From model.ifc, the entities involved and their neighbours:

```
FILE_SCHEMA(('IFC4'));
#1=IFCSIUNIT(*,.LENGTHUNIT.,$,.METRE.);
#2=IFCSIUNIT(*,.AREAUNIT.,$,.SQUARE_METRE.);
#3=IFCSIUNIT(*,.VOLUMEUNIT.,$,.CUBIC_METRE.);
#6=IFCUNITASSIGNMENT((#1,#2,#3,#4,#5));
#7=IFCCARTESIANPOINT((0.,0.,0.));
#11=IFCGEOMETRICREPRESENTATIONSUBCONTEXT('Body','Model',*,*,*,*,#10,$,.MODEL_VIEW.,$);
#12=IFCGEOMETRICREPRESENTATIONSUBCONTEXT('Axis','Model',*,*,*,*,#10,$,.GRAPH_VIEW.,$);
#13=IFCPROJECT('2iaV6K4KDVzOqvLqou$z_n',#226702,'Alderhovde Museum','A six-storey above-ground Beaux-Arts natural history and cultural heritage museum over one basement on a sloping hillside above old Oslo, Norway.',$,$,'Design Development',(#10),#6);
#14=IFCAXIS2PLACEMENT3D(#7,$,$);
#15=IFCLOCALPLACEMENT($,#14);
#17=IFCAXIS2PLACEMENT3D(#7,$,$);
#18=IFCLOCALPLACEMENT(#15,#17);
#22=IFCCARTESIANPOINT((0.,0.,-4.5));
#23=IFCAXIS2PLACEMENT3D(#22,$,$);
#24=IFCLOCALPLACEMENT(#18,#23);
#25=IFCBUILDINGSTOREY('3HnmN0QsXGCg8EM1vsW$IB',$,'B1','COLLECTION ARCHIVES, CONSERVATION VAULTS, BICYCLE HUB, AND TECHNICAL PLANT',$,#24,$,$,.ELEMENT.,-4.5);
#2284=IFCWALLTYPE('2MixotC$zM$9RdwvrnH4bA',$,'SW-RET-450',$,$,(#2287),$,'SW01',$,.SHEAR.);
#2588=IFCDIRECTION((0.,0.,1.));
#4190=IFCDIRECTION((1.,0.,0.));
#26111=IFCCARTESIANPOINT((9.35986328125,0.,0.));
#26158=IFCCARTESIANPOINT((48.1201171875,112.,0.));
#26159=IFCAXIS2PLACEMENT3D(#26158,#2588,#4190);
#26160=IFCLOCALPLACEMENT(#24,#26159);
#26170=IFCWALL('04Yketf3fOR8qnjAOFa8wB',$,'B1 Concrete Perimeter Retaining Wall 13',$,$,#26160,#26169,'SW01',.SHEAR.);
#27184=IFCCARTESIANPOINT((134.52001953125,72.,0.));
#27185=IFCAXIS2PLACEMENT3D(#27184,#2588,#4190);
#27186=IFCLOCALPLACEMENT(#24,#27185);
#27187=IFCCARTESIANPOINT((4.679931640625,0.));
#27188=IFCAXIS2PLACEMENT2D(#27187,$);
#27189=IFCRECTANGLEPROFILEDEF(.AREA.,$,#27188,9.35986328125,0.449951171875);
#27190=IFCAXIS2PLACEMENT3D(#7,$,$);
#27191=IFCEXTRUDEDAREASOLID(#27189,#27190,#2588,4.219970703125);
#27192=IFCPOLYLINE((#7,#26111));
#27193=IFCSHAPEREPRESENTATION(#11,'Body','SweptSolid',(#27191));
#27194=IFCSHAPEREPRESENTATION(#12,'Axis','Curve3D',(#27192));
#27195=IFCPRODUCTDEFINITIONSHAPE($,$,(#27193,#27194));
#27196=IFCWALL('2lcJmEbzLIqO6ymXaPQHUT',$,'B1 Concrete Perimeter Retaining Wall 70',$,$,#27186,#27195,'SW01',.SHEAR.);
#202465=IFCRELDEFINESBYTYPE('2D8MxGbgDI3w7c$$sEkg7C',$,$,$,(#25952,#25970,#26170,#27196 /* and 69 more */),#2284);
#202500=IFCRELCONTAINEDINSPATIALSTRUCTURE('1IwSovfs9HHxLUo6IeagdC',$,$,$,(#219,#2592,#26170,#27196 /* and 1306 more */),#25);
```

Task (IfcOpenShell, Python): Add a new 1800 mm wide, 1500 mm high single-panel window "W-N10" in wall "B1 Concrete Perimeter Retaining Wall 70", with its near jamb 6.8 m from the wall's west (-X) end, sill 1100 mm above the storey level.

```python
import numpy as np
import ifcopenshell
import ifcopenshell.api.feature
import ifcopenshell.api.geometry
import ifcopenshell.api.root
import ifcopenshell.api.spatial
import ifcopenshell.geom
import ifcopenshell.util.element
import ifcopenshell.util.placement
import ifcopenshell.util.representation
import ifcopenshell.util.shape
import ifcopenshell.util.unit

model = ifcopenshell.open("model.ifc")
unit_scale = ifcopenshell.util.unit.calculate_unit_scale(model)
settings = ifcopenshell.geom.settings()


def volume(element):
    """Net volume in cubic metres, openings subtracted."""
    shape = ifcopenshell.geom.create_shape(settings, element)
    return ifcopenshell.util.shape.get_volume(shape.geometry)


wall = model.by_guid("2lcJmEbzLIqO6ymXaPQHUT")
storey = ifcopenshell.util.element.get_container(wall, ifc_class="IfcBuildingStorey")
context = ifcopenshell.util.representation.get_context(model, "Model", "Body", "MODEL_VIEW")
before = volume(wall)

width, height, from_end, sill = 1.8, 1.5, 6.8, 1.1  # metres

# The wall runs along its own X axis, and the end named is its -X end.
wall_shape = ifcopenshell.geom.create_shape(settings, wall)
x, y, z = ifcopenshell.util.shape.get_vertices(wall_shape.geometry).T
start = x.min() + from_end
face, thickness = float(y.min()), float(y.max() - y.min())
wall_matrix = ifcopenshell.util.placement.get_local_placement(wall.ObjectPlacement)
level = ifcopenshell.util.placement.get_local_placement(storey.ObjectPlacement)[2, 3]


def in_wall(x, y):
    """Placement at x, y metres in the wall's axes, at sill height."""
    matrix = wall_matrix.copy()
    matrix[:, 3] = wall_matrix @ np.array([x / unit_scale, y / unit_scale, 0.0, 1.0])
    matrix[2, 3] = level + sill / unit_scale
    return matrix


# Opening: a box that overshoots both wall faces by 50 mm.
opening = ifcopenshell.api.root.create_entity(model, ifc_class="IfcOpeningElement", predefined_type="OPENING")
box = ifcopenshell.api.geometry.add_wall_representation(
    model, context=context, length=width, height=height, thickness=thickness + 0.1
)
ifcopenshell.api.geometry.assign_representation(model, product=opening, representation=box)
ifcopenshell.api.geometry.edit_object_placement(model, product=opening, matrix=in_wall(start, face - 0.05), is_si=False)
ifcopenshell.api.feature.add_feature(model, feature=opening, element=wall)

window = ifcopenshell.api.root.create_entity(model, ifc_class="IfcWindow", name="W-N10", predefined_type="WINDOW")
window.OverallWidth, window.OverallHeight = width / unit_scale, height / unit_scale
window.PartitioningType = "SINGLE_PANEL"
body = ifcopenshell.api.geometry.add_window_representation(
    model,
    context=context,
    overall_width=window.OverallWidth,
    overall_height=window.OverallHeight,
    partition_type="SINGLE_PANEL",
)
ifcopenshell.api.geometry.assign_representation(model, product=window, representation=body)
ifcopenshell.api.spatial.assign_container(model, products=[window], relating_structure=storey)
ifcopenshell.api.feature.add_filling(model, opening=opening, element=window)

# Centre the window in the wall's thickness.
ifcopenshell.api.geometry.edit_object_placement(model, product=window, matrix=in_wall(start, face), is_si=False)
window_shape = ifcopenshell.geom.create_shape(settings, window)
depth = ifcopenshell.util.shape.get_vertices(window_shape.geometry)[:, 1]
offset = face + thickness / 2 - (depth.min() + depth.max()) / 2
ifcopenshell.api.geometry.edit_object_placement(model, product=window, matrix=in_wall(start, offset), is_si=False)

after = volume(wall)

print(f"wall volume {before:.3f} -> {after:.3f} m3")

model.write("model_updated.ifc")
```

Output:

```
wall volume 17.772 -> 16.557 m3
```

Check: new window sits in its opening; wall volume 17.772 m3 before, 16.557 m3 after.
